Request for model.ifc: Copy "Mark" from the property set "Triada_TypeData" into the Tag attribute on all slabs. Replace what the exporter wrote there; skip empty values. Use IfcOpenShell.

First a look at what the model holds.

```python
import ifcopenshell
import ifcopenshell.util.element

model = ifcopenshell.open("model.ifc")
print(model.schema)
slabs = model.by_type("IfcSlab")
print(len(slabs), "slabs")
for e in slabs[:8]:
    source = ifcopenshell.util.element.get_pset(e, "Triada_TypeData", "Mark")
    target = e.Tag
    print(e.id(), repr(source), repr(target), sep=" | ")
```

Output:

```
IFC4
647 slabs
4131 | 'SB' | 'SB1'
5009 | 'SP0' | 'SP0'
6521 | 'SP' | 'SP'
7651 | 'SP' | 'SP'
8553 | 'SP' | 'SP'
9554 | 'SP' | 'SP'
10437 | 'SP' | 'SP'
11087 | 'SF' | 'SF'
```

```python
import ifcopenshell
import ifcopenshell.util.element

model = ifcopenshell.open("model.ifc")

count = 0
for e in model.by_type("IfcSlab"):
    value = ifcopenshell.util.element.get_pset(e, "Triada_TypeData", "Mark")
    current = e.Tag
    if not value or not value.strip() or current == value:
        continue
    e.Tag = value
    count += 1

print(count, "slabs updated")

model.write("model-out.ifc")
```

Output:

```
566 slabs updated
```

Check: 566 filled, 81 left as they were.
